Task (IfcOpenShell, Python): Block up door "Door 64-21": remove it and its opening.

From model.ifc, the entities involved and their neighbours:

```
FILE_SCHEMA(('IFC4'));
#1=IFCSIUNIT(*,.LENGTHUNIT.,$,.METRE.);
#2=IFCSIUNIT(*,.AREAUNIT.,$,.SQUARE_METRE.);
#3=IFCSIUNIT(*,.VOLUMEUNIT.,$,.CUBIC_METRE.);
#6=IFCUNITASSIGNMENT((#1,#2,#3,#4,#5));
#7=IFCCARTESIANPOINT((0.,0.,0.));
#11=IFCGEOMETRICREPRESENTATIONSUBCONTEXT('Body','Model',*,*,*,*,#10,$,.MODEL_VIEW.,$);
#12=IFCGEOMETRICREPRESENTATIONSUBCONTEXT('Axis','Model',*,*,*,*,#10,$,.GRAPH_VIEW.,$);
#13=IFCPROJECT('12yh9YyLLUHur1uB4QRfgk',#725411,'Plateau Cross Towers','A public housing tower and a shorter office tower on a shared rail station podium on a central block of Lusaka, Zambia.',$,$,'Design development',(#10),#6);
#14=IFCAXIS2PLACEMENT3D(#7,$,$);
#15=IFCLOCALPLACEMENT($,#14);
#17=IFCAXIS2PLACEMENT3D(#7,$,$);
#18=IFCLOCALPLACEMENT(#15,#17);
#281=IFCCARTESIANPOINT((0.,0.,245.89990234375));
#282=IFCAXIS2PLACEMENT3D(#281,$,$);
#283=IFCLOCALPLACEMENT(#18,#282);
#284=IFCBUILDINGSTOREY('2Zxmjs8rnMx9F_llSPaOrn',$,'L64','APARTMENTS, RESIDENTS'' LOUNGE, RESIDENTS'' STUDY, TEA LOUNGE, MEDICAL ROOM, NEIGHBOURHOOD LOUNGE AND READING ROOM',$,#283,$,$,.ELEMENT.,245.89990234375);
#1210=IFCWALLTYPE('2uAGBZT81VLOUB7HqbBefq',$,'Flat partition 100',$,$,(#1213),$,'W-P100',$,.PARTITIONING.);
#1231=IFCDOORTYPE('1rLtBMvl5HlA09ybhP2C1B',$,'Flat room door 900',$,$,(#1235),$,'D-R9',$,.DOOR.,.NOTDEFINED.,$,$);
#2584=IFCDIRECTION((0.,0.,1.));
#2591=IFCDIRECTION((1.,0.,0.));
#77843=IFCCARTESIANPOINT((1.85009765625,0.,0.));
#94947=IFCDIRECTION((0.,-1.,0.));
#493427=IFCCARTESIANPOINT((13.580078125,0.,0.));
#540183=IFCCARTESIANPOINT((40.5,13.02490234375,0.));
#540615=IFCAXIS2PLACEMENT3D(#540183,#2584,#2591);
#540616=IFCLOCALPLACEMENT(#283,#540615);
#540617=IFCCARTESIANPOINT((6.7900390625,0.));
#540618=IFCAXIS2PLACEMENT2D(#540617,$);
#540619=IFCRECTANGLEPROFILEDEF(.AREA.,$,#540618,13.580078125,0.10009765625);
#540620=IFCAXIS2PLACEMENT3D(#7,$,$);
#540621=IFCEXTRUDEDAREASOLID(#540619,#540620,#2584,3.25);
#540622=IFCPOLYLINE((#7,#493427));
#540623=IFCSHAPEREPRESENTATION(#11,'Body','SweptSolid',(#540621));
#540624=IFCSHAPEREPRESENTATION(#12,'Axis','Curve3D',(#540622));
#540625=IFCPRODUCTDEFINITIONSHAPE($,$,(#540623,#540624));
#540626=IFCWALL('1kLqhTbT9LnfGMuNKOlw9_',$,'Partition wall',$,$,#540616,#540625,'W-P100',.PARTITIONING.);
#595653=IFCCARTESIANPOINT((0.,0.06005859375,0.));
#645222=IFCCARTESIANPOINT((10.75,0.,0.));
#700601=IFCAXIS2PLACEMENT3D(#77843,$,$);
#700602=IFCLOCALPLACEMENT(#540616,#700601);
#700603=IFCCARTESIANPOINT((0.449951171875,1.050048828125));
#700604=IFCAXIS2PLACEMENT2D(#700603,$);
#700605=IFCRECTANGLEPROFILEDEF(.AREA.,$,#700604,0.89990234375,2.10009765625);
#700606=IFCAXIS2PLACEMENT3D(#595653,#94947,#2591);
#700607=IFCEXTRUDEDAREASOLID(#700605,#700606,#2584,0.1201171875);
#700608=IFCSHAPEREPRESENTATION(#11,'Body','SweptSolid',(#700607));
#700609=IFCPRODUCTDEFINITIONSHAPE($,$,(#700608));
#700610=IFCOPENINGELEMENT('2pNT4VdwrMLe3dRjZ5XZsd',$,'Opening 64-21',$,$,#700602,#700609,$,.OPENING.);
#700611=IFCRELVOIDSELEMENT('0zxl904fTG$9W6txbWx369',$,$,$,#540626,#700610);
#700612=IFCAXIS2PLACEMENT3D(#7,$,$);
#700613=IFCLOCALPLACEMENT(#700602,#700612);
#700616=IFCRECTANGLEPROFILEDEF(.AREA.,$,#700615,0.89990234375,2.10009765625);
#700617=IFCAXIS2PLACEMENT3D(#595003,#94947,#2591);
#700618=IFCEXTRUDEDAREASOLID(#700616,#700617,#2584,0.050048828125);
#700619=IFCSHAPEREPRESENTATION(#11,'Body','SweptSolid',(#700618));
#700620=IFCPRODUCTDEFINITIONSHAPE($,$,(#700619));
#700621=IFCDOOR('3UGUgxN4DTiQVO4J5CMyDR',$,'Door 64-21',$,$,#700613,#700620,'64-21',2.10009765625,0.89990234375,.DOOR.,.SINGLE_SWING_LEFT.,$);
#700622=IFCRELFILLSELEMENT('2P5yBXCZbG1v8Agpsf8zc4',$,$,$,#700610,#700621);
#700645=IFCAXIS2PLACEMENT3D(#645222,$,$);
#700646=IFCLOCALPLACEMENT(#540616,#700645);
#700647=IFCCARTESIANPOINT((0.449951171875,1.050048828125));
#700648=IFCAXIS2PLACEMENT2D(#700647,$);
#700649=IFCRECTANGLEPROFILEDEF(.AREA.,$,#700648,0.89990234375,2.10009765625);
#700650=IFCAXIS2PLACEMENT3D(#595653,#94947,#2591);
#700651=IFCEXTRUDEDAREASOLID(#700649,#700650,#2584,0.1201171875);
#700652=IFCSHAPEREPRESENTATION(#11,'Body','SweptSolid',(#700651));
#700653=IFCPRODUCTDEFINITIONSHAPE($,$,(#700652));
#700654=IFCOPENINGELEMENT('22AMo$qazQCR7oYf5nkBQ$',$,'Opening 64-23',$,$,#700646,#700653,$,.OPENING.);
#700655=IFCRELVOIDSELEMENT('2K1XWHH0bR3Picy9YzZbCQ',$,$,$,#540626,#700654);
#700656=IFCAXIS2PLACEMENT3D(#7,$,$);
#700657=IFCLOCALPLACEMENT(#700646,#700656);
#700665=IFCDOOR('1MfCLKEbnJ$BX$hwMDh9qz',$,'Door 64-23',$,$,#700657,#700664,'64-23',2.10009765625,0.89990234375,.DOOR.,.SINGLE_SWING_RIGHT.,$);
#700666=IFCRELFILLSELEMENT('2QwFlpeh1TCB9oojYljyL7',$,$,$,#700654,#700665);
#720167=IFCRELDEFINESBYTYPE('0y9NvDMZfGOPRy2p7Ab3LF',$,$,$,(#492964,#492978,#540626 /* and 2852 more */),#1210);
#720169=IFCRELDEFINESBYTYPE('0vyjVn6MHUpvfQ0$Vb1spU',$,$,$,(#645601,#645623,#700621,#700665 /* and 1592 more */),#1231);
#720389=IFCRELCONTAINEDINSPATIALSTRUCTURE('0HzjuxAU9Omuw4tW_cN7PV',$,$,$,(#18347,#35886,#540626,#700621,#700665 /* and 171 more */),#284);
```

```python
import ifcopenshell
import ifcopenshell.api.feature
import ifcopenshell.api.root
import ifcopenshell.geom
import ifcopenshell.util.shape

model = ifcopenshell.open("model.ifc")
settings = ifcopenshell.geom.settings()


def volume(element):
    """Net volume in cubic metres, openings subtracted."""
    shape = ifcopenshell.geom.create_shape(settings, element)
    return ifcopenshell.util.shape.get_volume(shape.geometry)


door = model.by_guid("3UGUgxN4DTiQVO4J5CMyDR")
opening = door.FillsVoids[0].RelatingOpeningElement
wall = opening.VoidsElements[0].RelatingBuildingElement
before = volume(wall)

ifcopenshell.api.root.remove_product(model, product=door)
ifcopenshell.api.feature.remove_feature(model, feature=opening)

after = volume(wall)

print(f"wall volume {before:.3f} -> {after:.3f} m3")

model.write("model-out.ifc")
```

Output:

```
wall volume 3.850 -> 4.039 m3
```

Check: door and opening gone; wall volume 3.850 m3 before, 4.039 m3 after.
